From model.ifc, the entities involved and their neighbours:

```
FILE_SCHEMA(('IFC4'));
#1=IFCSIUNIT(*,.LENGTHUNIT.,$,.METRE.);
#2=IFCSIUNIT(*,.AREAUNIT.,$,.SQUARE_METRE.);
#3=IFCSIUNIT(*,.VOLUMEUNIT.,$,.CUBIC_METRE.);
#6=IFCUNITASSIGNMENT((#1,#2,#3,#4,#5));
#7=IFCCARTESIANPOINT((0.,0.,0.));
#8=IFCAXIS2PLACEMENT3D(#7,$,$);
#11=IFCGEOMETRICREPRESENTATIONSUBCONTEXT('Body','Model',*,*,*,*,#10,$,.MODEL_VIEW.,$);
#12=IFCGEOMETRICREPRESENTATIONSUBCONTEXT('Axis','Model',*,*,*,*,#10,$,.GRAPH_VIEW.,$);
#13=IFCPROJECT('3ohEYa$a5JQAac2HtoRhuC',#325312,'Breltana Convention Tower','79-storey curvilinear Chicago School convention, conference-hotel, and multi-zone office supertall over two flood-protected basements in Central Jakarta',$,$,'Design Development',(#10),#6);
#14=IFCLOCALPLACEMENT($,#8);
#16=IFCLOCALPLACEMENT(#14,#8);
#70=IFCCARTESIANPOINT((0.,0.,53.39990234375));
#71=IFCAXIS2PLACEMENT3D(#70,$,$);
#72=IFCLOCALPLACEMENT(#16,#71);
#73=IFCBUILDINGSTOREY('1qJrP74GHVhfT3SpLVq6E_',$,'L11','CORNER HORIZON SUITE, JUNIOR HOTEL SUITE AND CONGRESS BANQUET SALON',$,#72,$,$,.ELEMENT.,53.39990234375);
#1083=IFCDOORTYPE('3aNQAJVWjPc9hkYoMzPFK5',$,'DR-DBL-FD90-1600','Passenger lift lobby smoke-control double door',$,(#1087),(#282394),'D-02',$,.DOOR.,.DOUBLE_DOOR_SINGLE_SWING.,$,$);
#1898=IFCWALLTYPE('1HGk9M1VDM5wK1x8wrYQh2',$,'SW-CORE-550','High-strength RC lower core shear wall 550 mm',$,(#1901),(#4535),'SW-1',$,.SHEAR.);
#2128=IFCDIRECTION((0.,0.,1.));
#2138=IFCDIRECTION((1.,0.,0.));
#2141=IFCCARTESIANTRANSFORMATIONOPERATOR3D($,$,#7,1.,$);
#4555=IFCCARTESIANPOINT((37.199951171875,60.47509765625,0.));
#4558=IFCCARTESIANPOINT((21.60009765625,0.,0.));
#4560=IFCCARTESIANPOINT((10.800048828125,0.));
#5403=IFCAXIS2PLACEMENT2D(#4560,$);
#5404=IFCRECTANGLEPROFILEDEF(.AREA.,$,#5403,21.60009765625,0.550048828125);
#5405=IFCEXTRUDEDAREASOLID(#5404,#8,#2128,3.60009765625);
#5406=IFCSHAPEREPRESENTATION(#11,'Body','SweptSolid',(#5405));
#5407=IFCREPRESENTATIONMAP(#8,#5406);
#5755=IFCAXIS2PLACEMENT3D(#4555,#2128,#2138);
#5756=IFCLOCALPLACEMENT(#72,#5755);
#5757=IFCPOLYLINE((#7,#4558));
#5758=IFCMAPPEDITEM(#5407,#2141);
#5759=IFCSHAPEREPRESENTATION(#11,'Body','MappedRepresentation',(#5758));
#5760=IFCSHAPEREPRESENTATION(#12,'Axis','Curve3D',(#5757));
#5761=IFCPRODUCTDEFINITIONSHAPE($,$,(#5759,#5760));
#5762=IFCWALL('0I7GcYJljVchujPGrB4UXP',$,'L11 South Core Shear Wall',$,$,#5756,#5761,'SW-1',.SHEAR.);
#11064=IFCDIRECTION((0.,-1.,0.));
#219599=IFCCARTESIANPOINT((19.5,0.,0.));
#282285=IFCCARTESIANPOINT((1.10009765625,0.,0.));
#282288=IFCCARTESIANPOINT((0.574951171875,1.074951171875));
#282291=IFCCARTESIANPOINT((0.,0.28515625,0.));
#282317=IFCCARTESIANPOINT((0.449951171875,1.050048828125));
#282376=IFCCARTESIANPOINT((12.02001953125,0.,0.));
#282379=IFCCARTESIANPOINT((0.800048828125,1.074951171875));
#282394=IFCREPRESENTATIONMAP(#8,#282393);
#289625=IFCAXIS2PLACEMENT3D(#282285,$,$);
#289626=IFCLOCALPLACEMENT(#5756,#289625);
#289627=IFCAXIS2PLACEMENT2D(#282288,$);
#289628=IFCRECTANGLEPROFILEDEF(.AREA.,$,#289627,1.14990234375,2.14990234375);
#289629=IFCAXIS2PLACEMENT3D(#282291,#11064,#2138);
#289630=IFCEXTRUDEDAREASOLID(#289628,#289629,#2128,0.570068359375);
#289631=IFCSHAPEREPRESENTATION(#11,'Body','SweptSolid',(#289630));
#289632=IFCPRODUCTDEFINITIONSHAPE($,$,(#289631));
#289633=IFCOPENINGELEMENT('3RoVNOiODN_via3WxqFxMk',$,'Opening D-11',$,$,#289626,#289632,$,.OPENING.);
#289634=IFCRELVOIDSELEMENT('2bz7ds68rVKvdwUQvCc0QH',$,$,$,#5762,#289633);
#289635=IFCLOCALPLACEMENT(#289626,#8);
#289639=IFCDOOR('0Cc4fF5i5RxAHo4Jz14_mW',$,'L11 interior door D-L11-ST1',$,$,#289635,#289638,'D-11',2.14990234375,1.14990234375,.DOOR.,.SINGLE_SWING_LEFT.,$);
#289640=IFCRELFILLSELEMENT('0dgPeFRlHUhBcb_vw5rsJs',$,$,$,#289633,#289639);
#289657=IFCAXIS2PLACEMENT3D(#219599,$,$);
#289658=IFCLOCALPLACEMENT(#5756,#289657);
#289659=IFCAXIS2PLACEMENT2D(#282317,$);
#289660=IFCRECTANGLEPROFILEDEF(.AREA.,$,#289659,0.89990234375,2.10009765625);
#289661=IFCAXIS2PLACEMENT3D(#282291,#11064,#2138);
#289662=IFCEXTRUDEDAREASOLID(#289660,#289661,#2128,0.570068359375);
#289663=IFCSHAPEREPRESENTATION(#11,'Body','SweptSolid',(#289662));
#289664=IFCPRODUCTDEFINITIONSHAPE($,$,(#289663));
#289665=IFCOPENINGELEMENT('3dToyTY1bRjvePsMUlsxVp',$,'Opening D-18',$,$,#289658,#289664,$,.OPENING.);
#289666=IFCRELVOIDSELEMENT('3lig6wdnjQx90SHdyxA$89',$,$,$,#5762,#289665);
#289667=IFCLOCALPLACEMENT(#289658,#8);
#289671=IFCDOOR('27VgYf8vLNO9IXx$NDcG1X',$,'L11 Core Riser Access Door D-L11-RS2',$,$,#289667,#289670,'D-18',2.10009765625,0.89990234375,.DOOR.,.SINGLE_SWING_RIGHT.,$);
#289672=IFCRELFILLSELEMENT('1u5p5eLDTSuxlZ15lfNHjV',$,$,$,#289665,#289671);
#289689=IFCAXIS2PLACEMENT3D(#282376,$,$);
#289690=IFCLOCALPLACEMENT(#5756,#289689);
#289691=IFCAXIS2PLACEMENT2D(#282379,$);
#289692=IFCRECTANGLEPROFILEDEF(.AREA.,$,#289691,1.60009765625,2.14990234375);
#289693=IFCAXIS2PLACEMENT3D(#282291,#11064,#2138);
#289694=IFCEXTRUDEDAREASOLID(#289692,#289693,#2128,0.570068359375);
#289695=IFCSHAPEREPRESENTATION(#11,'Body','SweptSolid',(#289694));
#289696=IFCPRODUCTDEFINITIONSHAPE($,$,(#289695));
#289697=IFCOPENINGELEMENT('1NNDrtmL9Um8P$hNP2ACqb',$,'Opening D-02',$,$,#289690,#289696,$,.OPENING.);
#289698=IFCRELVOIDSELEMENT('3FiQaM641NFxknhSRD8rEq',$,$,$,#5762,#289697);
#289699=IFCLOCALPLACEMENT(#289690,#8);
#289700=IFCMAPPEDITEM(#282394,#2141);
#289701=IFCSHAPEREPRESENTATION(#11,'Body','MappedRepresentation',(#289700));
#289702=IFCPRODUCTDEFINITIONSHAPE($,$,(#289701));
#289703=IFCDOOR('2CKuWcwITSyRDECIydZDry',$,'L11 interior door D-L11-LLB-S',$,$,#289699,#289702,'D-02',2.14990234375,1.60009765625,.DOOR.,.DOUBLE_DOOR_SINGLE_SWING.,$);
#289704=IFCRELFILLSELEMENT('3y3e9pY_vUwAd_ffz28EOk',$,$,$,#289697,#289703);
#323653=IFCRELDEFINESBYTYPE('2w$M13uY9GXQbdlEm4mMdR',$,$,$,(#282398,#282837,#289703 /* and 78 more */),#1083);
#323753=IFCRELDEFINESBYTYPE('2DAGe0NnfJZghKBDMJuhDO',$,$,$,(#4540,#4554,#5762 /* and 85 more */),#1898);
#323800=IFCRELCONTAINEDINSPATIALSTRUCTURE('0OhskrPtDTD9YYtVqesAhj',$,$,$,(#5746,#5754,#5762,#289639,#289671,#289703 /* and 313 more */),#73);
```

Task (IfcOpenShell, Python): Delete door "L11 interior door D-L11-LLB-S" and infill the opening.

```python
import ifcopenshell
import ifcopenshell.api.feature
import ifcopenshell.api.root
import ifcopenshell.geom
import ifcopenshell.util.shape

model = ifcopenshell.open("model.ifc")
settings = ifcopenshell.geom.settings()


def volume(element):
    """Net volume in cubic metres, openings subtracted."""
    shape = ifcopenshell.geom.create_shape(settings, element)
    return ifcopenshell.util.shape.get_volume(shape.geometry)


door = model.by_guid("2CKuWcwITSyRDECIydZDry")
opening = door.FillsVoids[0].RelatingOpeningElement
wall = opening.VoidsElements[0].RelatingBuildingElement
before = volume(wall)

ifcopenshell.api.root.remove_product(model, product=door)
ifcopenshell.api.feature.remove_feature(model, feature=opening)

after = volume(wall)

print(f"wall volume {before:.3f} -> {after:.3f} m3")

model.write("model_rev.ifc")
```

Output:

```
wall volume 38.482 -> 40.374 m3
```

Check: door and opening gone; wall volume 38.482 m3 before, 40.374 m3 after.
